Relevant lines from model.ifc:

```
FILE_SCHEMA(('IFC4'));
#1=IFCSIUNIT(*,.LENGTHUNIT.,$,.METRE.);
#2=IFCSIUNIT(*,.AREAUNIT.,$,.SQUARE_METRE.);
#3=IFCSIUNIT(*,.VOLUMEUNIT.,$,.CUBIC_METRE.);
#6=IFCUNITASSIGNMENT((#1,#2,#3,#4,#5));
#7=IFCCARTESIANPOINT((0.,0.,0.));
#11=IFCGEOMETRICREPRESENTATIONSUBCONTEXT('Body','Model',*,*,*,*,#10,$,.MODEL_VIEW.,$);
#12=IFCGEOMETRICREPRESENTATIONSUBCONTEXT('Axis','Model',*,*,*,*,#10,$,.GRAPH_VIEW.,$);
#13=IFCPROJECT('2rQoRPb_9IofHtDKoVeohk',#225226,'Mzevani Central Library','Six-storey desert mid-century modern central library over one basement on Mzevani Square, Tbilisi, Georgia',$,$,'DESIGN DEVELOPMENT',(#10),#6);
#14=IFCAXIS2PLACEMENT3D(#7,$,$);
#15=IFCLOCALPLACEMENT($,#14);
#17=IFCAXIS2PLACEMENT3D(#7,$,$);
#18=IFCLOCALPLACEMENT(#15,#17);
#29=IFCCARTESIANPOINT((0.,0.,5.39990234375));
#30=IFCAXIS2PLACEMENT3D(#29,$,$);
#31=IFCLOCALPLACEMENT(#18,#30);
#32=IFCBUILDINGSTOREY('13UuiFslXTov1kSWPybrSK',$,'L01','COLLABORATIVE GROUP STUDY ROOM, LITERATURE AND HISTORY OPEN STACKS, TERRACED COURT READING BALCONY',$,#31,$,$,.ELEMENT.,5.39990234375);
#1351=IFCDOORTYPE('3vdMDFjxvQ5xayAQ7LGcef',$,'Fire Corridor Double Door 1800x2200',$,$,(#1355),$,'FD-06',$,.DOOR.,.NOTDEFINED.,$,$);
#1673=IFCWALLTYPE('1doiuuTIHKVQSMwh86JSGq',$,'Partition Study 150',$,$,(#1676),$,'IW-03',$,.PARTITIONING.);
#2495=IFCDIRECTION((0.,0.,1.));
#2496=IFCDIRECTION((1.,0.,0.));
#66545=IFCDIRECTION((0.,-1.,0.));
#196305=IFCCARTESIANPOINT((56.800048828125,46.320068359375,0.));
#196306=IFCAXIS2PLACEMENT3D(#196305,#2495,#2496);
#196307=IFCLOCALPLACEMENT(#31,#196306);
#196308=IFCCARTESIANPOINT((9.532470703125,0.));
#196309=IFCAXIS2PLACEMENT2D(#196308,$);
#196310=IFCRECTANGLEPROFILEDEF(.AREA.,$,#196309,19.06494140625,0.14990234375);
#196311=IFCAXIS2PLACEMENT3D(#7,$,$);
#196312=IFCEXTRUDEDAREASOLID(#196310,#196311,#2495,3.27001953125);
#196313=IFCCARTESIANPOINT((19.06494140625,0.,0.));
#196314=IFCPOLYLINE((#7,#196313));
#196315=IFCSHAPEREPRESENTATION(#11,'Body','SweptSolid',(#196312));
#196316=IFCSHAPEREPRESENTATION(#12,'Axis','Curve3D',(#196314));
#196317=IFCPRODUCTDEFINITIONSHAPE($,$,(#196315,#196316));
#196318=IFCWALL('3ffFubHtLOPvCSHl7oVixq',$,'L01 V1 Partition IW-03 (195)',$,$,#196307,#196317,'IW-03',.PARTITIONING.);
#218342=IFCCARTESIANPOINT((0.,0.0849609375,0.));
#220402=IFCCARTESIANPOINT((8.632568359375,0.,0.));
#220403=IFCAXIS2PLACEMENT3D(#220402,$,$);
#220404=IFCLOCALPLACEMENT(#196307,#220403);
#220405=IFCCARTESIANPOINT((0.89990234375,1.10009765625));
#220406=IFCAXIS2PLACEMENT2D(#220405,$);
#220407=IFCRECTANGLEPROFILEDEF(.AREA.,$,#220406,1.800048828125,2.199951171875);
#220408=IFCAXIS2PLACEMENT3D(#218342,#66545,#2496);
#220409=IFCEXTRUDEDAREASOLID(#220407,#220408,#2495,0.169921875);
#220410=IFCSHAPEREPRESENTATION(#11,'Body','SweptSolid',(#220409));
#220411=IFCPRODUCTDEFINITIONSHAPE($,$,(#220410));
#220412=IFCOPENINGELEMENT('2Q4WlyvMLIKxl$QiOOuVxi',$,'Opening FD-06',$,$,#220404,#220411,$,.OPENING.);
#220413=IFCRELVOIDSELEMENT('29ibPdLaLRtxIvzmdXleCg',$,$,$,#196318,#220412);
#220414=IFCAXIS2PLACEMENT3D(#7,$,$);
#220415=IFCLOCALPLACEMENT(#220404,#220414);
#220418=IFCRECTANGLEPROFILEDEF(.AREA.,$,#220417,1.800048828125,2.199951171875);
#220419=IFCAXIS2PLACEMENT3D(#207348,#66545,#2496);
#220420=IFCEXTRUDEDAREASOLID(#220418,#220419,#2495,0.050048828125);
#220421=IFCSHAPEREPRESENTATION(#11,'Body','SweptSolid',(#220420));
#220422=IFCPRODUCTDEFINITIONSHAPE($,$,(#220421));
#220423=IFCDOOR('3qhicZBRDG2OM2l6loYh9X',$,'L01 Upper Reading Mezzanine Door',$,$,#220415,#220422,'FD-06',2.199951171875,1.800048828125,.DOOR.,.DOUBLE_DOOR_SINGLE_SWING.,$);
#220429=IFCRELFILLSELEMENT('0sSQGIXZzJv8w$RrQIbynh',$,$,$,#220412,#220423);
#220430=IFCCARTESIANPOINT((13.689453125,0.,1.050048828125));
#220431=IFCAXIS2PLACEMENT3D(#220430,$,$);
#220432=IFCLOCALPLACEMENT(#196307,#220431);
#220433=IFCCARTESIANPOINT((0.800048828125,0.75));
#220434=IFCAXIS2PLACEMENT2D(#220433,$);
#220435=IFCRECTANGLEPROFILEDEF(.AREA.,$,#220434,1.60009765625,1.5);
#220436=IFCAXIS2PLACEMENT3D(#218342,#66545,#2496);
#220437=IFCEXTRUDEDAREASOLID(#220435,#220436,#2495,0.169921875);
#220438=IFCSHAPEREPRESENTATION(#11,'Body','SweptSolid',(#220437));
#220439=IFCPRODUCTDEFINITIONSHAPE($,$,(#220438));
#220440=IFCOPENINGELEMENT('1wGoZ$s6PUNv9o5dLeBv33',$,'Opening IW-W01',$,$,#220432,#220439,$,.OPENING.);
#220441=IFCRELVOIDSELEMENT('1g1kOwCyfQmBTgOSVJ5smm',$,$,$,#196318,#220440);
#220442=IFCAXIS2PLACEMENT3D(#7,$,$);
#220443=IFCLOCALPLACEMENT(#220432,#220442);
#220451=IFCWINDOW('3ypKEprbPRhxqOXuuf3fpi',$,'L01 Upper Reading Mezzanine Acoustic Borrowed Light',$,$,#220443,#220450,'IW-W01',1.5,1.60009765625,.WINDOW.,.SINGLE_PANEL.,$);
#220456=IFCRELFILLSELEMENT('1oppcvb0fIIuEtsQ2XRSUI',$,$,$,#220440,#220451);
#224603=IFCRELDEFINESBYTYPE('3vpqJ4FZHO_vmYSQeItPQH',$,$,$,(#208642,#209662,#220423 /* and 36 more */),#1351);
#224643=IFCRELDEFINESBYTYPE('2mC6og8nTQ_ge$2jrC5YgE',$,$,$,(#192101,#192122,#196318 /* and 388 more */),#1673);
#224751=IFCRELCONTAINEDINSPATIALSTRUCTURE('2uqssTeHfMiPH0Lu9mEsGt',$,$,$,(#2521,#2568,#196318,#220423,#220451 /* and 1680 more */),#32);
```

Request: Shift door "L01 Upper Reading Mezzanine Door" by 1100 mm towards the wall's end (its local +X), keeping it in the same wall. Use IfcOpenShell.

```python
import ifcopenshell
import ifcopenshell.api.geometry
import ifcopenshell.util.placement
import ifcopenshell.util.unit

model = ifcopenshell.open("model.ifc")
unit_scale = ifcopenshell.util.unit.calculate_unit_scale(model)

door = model.by_guid("3qhicZBRDG2OM2l6loYh9X")
opening = door.FillsVoids[0].RelatingOpeningElement
wall = opening.VoidsElements[0].RelatingBuildingElement

wall_matrix = ifcopenshell.util.placement.get_local_placement(wall.ObjectPlacement)
shift = wall_matrix[:3, 0] * 1.1 / unit_scale
before = ifcopenshell.util.placement.get_local_placement(door.ObjectPlacement)[:3, 3].copy()

# The door is placed relative to its opening, so it follows when the opening moves.
matrix = ifcopenshell.util.placement.get_local_placement(opening.ObjectPlacement)
matrix[:3, 3] += shift
ifcopenshell.api.geometry.edit_object_placement(
    model, product=opening, matrix=matrix, is_si=False, should_transform_children=True
)

after = ifcopenshell.util.placement.get_local_placement(door.ObjectPlacement)[:3, 3]
print("door moved by", (after - before).round(3) + 0.0)

model.write("model_rev.ifc")
```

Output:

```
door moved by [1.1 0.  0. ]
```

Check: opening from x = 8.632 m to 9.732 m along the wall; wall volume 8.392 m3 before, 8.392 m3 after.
